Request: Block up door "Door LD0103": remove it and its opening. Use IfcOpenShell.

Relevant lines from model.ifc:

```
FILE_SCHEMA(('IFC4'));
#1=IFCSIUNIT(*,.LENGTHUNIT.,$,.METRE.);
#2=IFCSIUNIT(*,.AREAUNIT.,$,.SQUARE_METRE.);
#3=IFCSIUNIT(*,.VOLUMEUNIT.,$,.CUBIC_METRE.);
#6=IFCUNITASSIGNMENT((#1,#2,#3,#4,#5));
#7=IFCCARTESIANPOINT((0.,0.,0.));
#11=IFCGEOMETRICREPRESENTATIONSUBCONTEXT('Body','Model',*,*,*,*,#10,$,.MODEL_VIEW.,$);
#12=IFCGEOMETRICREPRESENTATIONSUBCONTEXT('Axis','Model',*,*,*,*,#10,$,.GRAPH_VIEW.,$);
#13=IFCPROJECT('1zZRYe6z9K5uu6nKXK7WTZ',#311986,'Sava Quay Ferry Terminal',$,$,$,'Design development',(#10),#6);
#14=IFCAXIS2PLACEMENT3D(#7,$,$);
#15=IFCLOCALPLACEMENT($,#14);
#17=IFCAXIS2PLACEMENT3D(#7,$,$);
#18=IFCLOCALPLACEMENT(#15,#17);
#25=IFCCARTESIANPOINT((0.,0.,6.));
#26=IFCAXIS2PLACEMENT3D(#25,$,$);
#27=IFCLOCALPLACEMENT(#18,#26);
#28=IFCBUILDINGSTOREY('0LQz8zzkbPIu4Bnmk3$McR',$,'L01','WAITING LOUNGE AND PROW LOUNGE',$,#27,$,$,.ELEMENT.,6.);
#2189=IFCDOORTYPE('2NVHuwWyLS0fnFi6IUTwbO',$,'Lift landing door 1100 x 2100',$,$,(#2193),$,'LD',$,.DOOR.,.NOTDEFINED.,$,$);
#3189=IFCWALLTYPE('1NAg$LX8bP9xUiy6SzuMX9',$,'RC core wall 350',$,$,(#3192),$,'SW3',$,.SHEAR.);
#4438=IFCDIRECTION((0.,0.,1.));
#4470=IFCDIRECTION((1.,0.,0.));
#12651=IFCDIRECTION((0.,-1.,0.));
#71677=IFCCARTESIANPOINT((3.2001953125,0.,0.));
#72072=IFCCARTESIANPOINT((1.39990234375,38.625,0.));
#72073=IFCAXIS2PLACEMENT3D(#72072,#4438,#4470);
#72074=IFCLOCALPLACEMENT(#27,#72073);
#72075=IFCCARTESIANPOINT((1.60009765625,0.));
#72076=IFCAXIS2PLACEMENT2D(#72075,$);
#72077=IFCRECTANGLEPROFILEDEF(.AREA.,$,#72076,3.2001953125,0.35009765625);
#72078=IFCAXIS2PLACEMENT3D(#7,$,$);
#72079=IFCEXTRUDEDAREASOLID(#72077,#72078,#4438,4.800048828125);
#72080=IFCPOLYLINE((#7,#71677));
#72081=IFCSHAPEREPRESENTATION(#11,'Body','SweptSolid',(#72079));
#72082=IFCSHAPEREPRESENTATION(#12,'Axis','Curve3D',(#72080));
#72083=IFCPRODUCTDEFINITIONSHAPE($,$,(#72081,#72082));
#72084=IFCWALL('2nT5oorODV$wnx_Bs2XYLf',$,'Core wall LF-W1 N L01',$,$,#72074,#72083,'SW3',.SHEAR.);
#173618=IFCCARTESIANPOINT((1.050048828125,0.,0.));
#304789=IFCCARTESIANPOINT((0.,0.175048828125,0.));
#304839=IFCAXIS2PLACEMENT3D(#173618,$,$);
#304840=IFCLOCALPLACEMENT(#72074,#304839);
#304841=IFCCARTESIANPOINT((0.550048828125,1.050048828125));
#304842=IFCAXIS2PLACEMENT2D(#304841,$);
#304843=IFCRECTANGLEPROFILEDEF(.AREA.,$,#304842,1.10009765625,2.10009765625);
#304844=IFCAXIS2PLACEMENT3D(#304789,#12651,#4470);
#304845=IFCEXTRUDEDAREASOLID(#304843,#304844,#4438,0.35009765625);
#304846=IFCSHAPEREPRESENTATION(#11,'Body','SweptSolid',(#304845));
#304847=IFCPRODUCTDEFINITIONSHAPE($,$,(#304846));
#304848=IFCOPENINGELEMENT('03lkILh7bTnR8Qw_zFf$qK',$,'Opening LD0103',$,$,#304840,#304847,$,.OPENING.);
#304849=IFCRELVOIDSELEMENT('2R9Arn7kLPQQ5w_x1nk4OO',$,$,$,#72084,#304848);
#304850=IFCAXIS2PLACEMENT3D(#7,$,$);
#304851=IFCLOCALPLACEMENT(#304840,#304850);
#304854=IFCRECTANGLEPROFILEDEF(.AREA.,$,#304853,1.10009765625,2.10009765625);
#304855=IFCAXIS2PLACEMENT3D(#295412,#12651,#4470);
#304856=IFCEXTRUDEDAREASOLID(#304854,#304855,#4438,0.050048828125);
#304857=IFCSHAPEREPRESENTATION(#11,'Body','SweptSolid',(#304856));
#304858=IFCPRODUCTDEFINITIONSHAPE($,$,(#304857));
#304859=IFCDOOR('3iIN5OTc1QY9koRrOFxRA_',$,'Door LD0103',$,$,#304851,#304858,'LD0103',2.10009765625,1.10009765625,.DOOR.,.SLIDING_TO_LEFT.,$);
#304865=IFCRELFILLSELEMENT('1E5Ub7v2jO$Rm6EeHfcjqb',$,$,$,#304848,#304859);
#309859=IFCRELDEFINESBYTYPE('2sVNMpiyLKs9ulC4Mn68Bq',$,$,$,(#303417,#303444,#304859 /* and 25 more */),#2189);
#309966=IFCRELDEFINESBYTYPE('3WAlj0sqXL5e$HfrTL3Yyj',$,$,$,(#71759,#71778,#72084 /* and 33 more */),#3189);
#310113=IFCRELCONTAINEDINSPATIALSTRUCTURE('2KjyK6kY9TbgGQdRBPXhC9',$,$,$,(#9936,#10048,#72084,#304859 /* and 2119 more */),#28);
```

```python
import ifcopenshell
import ifcopenshell.api.feature
import ifcopenshell.api.root
import ifcopenshell.geom
import ifcopenshell.util.shape

model = ifcopenshell.open("model.ifc")
settings = ifcopenshell.geom.settings()


def volume(element):
    """Net volume in cubic metres, openings subtracted."""
    shape = ifcopenshell.geom.create_shape(settings, element)
    return ifcopenshell.util.shape.get_volume(shape.geometry)


door = model.by_guid("3iIN5OTc1QY9koRrOFxRA_")
opening = door.FillsVoids[0].RelatingOpeningElement
wall = opening.VoidsElements[0].RelatingBuildingElement
before = volume(wall)

ifcopenshell.api.root.remove_product(model, product=door)
ifcopenshell.api.feature.remove_feature(model, feature=opening)

after = volume(wall)

print(f"wall volume {before:.3f} -> {after:.3f} m3")

model.write("model_v2.ifc")
```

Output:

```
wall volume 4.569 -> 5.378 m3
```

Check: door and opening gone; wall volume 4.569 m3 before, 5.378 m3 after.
